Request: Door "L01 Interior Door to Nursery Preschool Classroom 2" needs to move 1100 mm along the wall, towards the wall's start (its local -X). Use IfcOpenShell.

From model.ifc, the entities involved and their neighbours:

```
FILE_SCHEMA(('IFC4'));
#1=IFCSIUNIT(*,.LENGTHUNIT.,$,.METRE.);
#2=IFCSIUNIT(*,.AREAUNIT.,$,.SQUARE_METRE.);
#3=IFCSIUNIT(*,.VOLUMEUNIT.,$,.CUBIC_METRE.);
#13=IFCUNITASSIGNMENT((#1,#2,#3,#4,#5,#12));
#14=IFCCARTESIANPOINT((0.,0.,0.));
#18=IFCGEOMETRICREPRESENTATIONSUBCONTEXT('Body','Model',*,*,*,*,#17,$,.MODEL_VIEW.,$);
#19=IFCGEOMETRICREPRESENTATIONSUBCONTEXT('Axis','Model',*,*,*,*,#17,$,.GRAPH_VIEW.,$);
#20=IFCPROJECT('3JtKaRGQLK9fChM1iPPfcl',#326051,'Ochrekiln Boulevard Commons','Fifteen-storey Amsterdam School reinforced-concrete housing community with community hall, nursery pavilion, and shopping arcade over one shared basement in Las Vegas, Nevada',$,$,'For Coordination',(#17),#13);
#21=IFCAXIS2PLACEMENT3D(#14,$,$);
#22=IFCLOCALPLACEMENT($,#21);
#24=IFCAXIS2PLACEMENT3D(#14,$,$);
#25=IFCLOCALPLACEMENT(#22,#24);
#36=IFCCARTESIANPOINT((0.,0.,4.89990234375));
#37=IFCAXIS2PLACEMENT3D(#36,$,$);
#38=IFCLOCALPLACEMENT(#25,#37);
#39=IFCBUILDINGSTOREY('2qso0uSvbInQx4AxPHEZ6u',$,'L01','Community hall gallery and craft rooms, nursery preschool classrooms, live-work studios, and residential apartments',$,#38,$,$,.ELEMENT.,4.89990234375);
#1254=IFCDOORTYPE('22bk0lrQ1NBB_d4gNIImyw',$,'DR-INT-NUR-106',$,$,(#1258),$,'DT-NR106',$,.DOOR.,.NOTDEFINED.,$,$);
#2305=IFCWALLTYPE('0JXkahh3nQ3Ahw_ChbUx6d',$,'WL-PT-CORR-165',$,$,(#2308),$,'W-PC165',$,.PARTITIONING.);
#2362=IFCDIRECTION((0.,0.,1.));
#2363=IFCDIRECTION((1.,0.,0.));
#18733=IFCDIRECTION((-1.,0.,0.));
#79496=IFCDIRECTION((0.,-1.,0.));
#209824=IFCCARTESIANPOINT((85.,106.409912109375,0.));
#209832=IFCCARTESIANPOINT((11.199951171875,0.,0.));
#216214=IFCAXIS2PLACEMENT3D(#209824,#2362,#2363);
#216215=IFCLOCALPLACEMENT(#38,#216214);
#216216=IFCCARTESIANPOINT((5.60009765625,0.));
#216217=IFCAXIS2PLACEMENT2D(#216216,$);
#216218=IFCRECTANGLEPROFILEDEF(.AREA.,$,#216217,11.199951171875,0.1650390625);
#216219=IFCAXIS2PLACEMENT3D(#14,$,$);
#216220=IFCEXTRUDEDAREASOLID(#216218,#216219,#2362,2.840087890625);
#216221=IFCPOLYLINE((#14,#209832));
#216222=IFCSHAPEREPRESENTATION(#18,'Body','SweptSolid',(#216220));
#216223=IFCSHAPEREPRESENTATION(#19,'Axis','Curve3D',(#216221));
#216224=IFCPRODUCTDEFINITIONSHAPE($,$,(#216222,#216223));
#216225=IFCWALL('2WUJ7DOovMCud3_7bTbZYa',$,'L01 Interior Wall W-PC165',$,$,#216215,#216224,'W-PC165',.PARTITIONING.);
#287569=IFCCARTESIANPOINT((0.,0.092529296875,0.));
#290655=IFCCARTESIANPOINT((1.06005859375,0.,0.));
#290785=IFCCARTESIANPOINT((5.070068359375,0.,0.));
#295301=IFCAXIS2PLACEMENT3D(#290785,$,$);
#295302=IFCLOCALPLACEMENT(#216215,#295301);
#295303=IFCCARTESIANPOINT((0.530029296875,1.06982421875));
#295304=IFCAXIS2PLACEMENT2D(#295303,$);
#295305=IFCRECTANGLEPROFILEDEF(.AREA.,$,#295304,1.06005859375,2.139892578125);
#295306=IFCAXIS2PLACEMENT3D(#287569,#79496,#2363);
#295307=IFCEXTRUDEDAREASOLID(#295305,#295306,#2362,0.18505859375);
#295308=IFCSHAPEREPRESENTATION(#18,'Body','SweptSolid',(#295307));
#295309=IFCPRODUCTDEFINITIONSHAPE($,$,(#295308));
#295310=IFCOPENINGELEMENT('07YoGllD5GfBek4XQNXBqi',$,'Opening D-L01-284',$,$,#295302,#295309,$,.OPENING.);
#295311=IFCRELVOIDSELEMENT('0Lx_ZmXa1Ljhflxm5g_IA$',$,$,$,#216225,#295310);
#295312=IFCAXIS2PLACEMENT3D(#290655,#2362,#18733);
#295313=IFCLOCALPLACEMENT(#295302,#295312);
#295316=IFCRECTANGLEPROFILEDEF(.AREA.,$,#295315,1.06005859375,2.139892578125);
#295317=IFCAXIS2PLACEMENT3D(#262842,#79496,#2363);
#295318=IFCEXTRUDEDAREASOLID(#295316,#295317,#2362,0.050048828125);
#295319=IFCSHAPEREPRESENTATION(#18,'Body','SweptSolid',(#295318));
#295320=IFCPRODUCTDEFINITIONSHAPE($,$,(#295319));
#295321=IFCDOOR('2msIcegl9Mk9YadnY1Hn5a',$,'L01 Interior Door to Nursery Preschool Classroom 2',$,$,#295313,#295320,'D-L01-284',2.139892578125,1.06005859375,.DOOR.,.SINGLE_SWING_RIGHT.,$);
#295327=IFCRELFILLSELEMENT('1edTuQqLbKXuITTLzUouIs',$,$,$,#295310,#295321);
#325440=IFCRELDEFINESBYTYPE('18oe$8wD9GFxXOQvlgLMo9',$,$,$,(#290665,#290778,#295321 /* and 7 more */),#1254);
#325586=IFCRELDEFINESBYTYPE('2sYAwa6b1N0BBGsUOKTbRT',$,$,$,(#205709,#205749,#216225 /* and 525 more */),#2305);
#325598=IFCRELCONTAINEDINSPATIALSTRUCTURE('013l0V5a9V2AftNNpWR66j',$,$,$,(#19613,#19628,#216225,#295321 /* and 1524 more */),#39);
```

```python
import ifcopenshell
import ifcopenshell.api.geometry
import ifcopenshell.util.placement

model = ifcopenshell.open("model.ifc")

door = model.by_id(295321)
opening = door.FillsVoids[0].RelatingOpeningElement
wall = opening.VoidsElements[0].RelatingBuildingElement

wall_matrix = ifcopenshell.util.placement.get_local_placement(wall.ObjectPlacement)
shift = wall_matrix[:3, 0] * -1.1
before = ifcopenshell.util.placement.get_local_placement(door.ObjectPlacement)[:3, 3].copy()

# The door is placed relative to its opening, so it follows when the opening moves.
matrix = ifcopenshell.util.placement.get_local_placement(opening.ObjectPlacement)
matrix[:3, 3] += shift
ifcopenshell.api.geometry.edit_object_placement(
    model, product=opening, matrix=matrix, is_si=False, should_transform_children=True
)

after = ifcopenshell.util.placement.get_local_placement(door.ObjectPlacement)[:3, 3]
print("door moved by", (after - before).round(3) + 0.0)

model.write("model_updated.ifc")
```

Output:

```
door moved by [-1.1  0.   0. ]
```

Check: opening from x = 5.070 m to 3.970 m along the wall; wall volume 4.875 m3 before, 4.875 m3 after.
